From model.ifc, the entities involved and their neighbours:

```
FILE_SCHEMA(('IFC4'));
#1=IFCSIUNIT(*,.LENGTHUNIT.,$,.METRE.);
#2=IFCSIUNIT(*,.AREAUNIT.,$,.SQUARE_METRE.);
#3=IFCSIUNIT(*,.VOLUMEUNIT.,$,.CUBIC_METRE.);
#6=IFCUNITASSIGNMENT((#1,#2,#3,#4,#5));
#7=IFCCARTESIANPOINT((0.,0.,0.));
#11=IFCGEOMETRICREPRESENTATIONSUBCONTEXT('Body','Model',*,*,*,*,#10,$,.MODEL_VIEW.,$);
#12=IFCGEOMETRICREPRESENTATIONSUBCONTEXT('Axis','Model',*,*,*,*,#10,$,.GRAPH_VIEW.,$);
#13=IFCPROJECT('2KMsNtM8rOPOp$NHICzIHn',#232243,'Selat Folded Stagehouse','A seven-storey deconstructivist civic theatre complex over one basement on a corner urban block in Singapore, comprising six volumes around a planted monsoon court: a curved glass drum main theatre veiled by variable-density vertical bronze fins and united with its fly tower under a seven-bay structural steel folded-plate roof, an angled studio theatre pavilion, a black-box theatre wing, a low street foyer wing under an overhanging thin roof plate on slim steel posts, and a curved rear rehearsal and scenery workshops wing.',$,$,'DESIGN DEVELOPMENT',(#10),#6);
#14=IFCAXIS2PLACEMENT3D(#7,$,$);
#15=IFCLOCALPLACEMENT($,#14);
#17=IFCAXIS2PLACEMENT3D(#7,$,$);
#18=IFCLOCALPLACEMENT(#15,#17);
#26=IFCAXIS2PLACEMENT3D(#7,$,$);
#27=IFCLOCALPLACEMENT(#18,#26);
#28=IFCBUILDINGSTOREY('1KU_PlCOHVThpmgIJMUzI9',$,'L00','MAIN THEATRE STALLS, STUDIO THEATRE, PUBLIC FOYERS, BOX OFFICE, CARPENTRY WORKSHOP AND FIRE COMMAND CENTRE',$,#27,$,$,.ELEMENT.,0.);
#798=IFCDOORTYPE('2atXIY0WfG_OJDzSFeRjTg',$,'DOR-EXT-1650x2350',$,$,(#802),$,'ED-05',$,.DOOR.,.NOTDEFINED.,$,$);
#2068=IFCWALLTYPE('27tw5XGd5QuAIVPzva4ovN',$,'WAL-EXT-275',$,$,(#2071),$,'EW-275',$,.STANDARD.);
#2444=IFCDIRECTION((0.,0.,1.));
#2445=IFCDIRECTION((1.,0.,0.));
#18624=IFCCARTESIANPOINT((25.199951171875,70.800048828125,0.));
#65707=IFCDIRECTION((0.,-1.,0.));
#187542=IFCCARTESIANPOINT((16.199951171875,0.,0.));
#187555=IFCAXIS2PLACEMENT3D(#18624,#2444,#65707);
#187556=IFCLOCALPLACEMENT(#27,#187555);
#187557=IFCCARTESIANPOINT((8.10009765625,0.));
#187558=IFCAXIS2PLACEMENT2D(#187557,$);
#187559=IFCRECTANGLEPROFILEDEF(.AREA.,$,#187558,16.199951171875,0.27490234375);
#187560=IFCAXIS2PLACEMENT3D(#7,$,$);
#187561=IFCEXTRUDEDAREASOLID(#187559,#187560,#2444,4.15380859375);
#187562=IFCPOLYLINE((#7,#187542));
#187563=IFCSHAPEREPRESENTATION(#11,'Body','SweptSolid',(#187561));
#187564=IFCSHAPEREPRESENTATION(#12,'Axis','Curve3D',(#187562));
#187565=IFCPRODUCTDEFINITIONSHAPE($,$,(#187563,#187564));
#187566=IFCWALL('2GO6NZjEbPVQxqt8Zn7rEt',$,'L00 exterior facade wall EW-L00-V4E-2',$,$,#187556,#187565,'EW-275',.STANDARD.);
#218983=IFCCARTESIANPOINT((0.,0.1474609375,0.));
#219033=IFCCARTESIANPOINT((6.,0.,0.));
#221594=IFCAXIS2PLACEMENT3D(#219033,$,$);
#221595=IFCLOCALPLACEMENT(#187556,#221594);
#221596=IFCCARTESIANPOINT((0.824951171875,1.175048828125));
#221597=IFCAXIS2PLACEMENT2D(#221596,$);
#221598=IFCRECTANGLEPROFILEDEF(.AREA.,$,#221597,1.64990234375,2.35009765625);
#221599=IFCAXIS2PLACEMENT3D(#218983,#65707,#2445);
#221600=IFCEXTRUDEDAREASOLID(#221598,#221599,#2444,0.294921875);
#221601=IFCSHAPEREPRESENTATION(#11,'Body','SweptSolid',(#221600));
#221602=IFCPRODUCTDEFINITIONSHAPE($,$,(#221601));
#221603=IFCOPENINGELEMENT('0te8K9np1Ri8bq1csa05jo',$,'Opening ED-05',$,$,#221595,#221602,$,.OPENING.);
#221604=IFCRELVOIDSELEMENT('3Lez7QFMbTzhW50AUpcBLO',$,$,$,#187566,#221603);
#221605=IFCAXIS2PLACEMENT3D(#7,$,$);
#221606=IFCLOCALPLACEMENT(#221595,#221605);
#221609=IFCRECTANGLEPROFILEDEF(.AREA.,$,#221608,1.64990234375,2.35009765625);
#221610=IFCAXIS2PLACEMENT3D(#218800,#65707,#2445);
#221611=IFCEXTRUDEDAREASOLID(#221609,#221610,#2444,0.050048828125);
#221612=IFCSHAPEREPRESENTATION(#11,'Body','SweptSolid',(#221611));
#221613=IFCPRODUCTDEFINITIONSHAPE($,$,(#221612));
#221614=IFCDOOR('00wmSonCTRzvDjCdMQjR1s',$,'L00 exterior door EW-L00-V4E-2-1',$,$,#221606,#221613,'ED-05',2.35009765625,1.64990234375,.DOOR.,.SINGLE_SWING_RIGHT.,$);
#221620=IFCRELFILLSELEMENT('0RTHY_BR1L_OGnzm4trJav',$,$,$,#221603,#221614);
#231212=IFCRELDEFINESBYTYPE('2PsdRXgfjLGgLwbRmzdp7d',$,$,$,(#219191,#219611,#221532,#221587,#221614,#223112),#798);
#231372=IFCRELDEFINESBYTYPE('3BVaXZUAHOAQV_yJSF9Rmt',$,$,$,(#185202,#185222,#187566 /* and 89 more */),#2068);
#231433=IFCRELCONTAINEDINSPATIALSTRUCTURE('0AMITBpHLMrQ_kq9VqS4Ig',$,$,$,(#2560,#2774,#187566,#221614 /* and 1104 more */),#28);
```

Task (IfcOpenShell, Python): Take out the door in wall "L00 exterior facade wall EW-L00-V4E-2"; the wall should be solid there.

```python
import ifcopenshell
import ifcopenshell.api.feature
import ifcopenshell.api.root
import ifcopenshell.geom
import ifcopenshell.util.shape

model = ifcopenshell.open("model.ifc")
settings = ifcopenshell.geom.settings()


def volume(element):
    """Net volume in cubic metres, openings subtracted."""
    shape = ifcopenshell.geom.create_shape(settings, element)
    return ifcopenshell.util.shape.get_volume(shape.geometry)


door = model.by_guid("00wmSonCTRzvDjCdMQjR1s")
opening = door.FillsVoids[0].RelatingOpeningElement
wall = opening.VoidsElements[0].RelatingBuildingElement
before = volume(wall)

ifcopenshell.api.root.remove_product(model, product=door)
ifcopenshell.api.feature.remove_feature(model, feature=opening)

after = volume(wall)

print(f"wall volume {before:.3f} -> {after:.3f} m3")

model.write("model_v2.ifc")
```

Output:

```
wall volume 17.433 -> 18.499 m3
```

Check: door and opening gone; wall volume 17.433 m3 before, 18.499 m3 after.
